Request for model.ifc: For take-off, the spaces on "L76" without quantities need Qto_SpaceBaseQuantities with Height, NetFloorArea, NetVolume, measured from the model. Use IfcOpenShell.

First a look at what the model holds.

```python
import ifcopenshell
import ifcopenshell.util.element
import ifcopenshell.util.unit

model = ifcopenshell.open("model.ifc")
print(model.schema)
for unit_type in ("LENGTHUNIT", "AREAUNIT", "VOLUMEUNIT"):
    print(unit_type, ifcopenshell.util.unit.calculate_unit_scale(model, unit_type))
storey = next(s for s in model.by_type("IfcBuildingStorey") if s.Name == "L76")
spaces = [e for e in ifcopenshell.util.element.get_decomposition(storey) if e.is_a("IfcSpace")]
for e in sorted(spaces, key=lambda e: e.id()):
    print(e.id(), e.is_a(), e.Name, list(ifcopenshell.util.element.get_psets(e, qtos_only=True)), sep=" | ")
```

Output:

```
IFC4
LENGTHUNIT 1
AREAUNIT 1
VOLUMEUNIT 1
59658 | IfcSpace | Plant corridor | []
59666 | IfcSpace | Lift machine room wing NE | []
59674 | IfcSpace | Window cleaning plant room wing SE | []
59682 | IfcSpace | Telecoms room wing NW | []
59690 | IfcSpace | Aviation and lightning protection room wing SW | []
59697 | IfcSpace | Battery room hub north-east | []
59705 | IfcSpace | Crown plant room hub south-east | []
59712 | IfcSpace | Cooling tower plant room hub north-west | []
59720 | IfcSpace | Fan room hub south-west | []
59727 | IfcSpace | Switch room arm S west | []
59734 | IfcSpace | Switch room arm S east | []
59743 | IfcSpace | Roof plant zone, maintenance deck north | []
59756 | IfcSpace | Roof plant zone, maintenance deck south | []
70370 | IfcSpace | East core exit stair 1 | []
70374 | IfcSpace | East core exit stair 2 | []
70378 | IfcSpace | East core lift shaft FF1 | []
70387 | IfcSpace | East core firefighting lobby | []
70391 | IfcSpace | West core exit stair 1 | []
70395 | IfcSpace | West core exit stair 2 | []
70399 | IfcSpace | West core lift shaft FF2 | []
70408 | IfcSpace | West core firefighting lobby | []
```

```python
import ifcopenshell
import ifcopenshell.api.pset
import ifcopenshell.geom
import ifcopenshell.util.element
import ifcopenshell.util.shape
import ifcopenshell.util.unit

model = ifcopenshell.open("model.ifc")
unit_scale = ifcopenshell.util.unit.calculate_unit_scale(model)
area_scale = ifcopenshell.util.unit.calculate_unit_scale(model, "AREAUNIT")
volume_scale = ifcopenshell.util.unit.calculate_unit_scale(model, "VOLUMEUNIT")
settings = ifcopenshell.geom.settings()

storey = next(s for s in model.by_type("IfcBuildingStorey") if s.Name == "L76")
spaces = [e for e in ifcopenshell.util.element.get_decomposition(storey) if e.is_a("IfcSpace")]

for e in sorted(spaces, key=lambda e: e.id()):
    if ifcopenshell.util.element.get_psets(e, qtos_only=True, should_inherit=False):
        continue
    # Geometry comes back in metres, in the element's own axes.
    shape = ifcopenshell.geom.create_shape(settings, e)
    values = {
        "Height": ifcopenshell.util.shape.get_z(shape.geometry) / unit_scale,
        "NetFloorArea": ifcopenshell.util.shape.get_footprint_area(shape.geometry) / area_scale,
        "NetVolume": ifcopenshell.util.shape.get_volume(shape.geometry) / volume_scale,
    }
    qto = ifcopenshell.api.pset.add_qto(model, product=e, name="Qto_SpaceBaseQuantities")
    ifcopenshell.api.pset.edit_qto(model, qto=qto, properties=values)
    print(e.id(), {k: round(v, 3) for k, v in values.items()})

model.write("model_edited.ifc")
```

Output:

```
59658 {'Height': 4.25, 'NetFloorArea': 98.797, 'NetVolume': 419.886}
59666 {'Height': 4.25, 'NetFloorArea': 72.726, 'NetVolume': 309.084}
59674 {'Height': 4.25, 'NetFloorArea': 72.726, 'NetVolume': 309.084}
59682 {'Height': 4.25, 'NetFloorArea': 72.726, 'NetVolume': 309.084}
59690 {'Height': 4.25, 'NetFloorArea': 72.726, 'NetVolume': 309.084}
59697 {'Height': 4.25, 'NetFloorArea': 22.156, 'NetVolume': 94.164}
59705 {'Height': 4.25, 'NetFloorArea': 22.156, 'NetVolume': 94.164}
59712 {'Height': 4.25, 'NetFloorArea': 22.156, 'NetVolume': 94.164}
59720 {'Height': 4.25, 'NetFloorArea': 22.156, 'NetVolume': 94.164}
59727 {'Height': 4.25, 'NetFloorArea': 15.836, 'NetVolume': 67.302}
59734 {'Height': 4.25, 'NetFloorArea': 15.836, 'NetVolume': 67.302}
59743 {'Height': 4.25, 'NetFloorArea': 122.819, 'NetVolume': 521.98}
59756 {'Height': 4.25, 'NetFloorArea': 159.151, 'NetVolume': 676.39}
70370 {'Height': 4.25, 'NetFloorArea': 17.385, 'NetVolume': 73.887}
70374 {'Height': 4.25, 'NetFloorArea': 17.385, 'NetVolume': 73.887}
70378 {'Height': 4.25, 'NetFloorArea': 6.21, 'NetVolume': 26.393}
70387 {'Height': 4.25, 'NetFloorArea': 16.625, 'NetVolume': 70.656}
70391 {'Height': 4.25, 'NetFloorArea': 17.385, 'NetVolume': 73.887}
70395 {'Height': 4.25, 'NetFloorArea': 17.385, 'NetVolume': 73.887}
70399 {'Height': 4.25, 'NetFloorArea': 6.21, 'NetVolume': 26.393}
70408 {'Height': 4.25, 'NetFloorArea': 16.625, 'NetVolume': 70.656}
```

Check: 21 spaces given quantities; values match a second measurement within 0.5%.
